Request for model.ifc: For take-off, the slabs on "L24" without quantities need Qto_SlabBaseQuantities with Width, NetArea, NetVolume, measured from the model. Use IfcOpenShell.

First a look at what the model holds.

```python
import ifcopenshell
import ifcopenshell.util.element
import ifcopenshell.util.unit

model = ifcopenshell.open("model.ifc")
print(model.schema)
for unit_type in ("LENGTHUNIT", "AREAUNIT", "VOLUMEUNIT"):
    print(unit_type, ifcopenshell.util.unit.calculate_unit_scale(model, unit_type))
storey = next(s for s in model.by_type("IfcBuildingStorey") if s.Name == "L24")
slabs = [e for e in ifcopenshell.util.element.get_decomposition(storey) if e.is_a("IfcSlab")]
for e in sorted(slabs, key=lambda e: e.id()):
    print(e.id(), e.is_a(), e.Name, list(ifcopenshell.util.element.get_psets(e, qtos_only=True)), sep=" | ")
```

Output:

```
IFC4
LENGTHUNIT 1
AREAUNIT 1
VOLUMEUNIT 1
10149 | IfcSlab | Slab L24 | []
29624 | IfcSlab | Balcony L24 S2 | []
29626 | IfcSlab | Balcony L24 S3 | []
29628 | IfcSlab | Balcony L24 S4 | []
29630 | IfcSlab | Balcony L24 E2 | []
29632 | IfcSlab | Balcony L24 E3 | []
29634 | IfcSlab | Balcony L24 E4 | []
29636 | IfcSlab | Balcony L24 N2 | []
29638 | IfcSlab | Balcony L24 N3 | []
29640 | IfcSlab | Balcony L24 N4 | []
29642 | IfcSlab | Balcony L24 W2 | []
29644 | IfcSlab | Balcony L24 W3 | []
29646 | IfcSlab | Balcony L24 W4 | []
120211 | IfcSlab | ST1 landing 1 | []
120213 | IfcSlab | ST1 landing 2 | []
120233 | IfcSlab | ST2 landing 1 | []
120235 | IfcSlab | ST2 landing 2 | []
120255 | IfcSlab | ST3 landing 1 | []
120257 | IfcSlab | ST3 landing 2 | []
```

```python
import ifcopenshell
import ifcopenshell.api.pset
import ifcopenshell.geom
import ifcopenshell.util.element
import ifcopenshell.util.shape
import ifcopenshell.util.unit

model = ifcopenshell.open("model.ifc")
unit_scale = ifcopenshell.util.unit.calculate_unit_scale(model)
area_scale = ifcopenshell.util.unit.calculate_unit_scale(model, "AREAUNIT")
volume_scale = ifcopenshell.util.unit.calculate_unit_scale(model, "VOLUMEUNIT")
settings = ifcopenshell.geom.settings()

storey = next(s for s in model.by_type("IfcBuildingStorey") if s.Name == "L24")
slabs = [e for e in ifcopenshell.util.element.get_decomposition(storey) if e.is_a("IfcSlab")]

for e in sorted(slabs, key=lambda e: e.id()):
    if ifcopenshell.util.element.get_psets(e, qtos_only=True, should_inherit=False):
        continue
    # Geometry comes back in metres, in the element's own axes.
    shape = ifcopenshell.geom.create_shape(settings, e)
    values = {
        "Width": ifcopenshell.util.shape.get_z(shape.geometry) / unit_scale,
        "NetArea": ifcopenshell.util.shape.get_footprint_area(shape.geometry) / area_scale,
        "NetVolume": ifcopenshell.util.shape.get_volume(shape.geometry) / volume_scale,
    }
    qto = ifcopenshell.api.pset.add_qto(model, product=e, name="Qto_SlabBaseQuantities")
    ifcopenshell.api.pset.edit_qto(model, qto=qto, properties=values)
    print(e.id(), {k: round(v, 3) for k, v in values.items()})

model.write("model-out.ifc")
```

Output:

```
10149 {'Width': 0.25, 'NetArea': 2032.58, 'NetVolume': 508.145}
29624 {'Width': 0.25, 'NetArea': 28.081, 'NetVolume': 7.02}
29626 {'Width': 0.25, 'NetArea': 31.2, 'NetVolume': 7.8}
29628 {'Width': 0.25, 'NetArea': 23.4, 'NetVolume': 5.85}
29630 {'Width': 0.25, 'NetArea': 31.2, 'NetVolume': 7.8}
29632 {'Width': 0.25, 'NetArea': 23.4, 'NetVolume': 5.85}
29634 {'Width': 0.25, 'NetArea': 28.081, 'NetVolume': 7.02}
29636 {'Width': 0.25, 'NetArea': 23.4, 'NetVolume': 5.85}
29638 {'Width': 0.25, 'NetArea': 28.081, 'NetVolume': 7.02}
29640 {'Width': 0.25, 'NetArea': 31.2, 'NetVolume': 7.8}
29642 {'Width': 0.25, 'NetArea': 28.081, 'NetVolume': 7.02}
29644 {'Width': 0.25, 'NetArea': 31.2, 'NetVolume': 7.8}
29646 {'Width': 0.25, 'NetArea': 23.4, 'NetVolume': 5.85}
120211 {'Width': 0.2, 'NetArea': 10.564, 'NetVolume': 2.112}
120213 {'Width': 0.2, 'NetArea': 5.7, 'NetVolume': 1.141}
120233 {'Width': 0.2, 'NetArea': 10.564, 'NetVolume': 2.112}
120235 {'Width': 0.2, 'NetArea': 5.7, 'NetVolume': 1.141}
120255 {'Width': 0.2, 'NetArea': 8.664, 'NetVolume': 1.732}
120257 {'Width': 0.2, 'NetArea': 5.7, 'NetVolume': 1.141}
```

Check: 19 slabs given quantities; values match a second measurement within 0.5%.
